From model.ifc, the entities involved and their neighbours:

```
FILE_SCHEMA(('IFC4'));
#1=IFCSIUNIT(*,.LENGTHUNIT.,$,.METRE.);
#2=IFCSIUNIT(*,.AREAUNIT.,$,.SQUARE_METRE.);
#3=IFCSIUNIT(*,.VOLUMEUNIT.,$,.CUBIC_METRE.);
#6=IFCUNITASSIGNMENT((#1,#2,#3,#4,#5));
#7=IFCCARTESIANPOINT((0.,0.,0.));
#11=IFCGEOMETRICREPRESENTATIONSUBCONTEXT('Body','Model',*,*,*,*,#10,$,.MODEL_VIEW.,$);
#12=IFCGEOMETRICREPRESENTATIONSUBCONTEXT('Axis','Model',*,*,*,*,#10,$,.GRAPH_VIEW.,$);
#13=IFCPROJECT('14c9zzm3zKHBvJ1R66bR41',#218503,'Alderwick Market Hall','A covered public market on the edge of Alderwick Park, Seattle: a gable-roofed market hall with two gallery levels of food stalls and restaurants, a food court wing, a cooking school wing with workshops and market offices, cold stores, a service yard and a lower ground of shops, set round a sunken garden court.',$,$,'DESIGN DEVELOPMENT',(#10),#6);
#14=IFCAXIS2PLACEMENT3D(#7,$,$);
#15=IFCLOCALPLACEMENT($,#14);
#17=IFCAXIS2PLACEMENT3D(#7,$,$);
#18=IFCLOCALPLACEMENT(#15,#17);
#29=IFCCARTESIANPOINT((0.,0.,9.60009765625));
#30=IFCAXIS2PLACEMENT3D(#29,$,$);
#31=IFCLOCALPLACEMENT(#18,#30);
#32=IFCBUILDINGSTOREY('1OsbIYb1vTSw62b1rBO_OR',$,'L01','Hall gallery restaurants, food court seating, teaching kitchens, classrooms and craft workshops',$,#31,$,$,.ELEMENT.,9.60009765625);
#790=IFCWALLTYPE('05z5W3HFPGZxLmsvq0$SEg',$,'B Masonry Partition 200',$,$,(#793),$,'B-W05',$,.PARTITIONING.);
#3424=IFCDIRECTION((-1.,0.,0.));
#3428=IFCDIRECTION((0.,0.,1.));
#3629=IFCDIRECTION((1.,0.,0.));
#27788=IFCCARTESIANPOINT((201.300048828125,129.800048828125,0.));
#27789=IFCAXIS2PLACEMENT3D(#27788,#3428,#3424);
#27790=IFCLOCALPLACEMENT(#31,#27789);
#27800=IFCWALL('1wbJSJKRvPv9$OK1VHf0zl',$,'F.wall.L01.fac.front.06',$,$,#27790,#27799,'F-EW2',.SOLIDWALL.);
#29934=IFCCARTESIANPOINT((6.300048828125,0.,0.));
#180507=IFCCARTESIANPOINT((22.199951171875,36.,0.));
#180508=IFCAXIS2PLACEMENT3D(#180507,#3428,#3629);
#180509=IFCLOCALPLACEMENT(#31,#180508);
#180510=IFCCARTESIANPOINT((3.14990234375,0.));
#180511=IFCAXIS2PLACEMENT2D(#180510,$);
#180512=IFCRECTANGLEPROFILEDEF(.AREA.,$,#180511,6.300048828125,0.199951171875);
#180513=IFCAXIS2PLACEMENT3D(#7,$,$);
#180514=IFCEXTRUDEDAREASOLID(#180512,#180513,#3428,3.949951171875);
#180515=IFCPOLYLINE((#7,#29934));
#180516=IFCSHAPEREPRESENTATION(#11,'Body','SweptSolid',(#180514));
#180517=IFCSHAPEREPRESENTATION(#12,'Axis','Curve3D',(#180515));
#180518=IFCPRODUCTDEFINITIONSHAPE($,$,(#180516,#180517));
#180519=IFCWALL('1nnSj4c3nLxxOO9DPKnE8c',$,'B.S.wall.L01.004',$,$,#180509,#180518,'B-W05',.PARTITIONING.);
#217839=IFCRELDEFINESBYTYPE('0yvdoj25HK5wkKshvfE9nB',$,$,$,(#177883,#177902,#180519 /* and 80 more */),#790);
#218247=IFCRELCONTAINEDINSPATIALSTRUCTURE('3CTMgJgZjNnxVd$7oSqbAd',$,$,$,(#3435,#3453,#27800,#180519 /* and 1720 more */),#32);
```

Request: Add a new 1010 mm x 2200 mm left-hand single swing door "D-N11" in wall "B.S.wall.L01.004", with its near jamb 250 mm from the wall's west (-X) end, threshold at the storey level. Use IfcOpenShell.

```python
import numpy as np
import ifcopenshell
import ifcopenshell.api.feature
import ifcopenshell.api.geometry
import ifcopenshell.api.root
import ifcopenshell.api.spatial
import ifcopenshell.geom
import ifcopenshell.util.element
import ifcopenshell.util.placement
import ifcopenshell.util.representation
import ifcopenshell.util.shape
import ifcopenshell.util.unit

model = ifcopenshell.open("model.ifc")
unit_scale = ifcopenshell.util.unit.calculate_unit_scale(model)
settings = ifcopenshell.geom.settings()


def volume(element):
    """Net volume in cubic metres, openings subtracted."""
    shape = ifcopenshell.geom.create_shape(settings, element)
    return ifcopenshell.util.shape.get_volume(shape.geometry)


wall = model.by_guid("1nnSj4c3nLxxOO9DPKnE8c")
storey = ifcopenshell.util.element.get_container(wall, ifc_class="IfcBuildingStorey")
context = ifcopenshell.util.representation.get_context(model, "Model", "Body", "MODEL_VIEW")
before = volume(wall)

width, height, from_end, sill = 1.01, 2.2, 0.25, 0.0  # metres

# The wall runs along its own X axis, and the end named is its -X end.
wall_shape = ifcopenshell.geom.create_shape(settings, wall)
x, y, z = ifcopenshell.util.shape.get_vertices(wall_shape.geometry).T
start = x.min() + from_end
face, thickness = float(y.min()), float(y.max() - y.min())
wall_matrix = ifcopenshell.util.placement.get_local_placement(wall.ObjectPlacement)
level = ifcopenshell.util.placement.get_local_placement(storey.ObjectPlacement)[2, 3]


def in_wall(x, y):
    """Placement at x, y metres in the wall's axes, at sill height."""
    matrix = wall_matrix.copy()
    matrix[:, 3] = wall_matrix @ np.array([x / unit_scale, y / unit_scale, 0.0, 1.0])
    matrix[2, 3] = level + sill / unit_scale
    return matrix


# Opening: a box that overshoots both wall faces by 50 mm.
opening = ifcopenshell.api.root.create_entity(model, ifc_class="IfcOpeningElement", predefined_type="OPENING")
box = ifcopenshell.api.geometry.add_wall_representation(
    model, context=context, length=width, height=height, thickness=thickness + 0.1
)
ifcopenshell.api.geometry.assign_representation(model, product=opening, representation=box)
ifcopenshell.api.geometry.edit_object_placement(model, product=opening, matrix=in_wall(start, face - 0.05), is_si=False)
ifcopenshell.api.feature.add_feature(model, feature=opening, element=wall)

door = ifcopenshell.api.root.create_entity(model, ifc_class="IfcDoor", name="D-N11", predefined_type="DOOR")
door.OverallWidth, door.OverallHeight = width / unit_scale, height / unit_scale
door.OperationType = "SINGLE_SWING_LEFT"
body = ifcopenshell.api.geometry.add_door_representation(
    model,
    context=context,
    overall_width=door.OverallWidth,
    overall_height=door.OverallHeight,
    operation_type="SINGLE_SWING_LEFT",
    lining_properties={"LiningDepth": thickness / unit_scale, "ThresholdDepth": thickness / unit_scale},
)
ifcopenshell.api.geometry.assign_representation(model, product=door, representation=body)
ifcopenshell.api.spatial.assign_container(model, products=[door], relating_structure=storey)
ifcopenshell.api.feature.add_filling(model, opening=opening, element=door)

# The lining spans the wall, so the door starts at the wall face.
ifcopenshell.api.geometry.edit_object_placement(model, product=door, matrix=in_wall(start, face), is_si=False)

after = volume(wall)

print(f"wall volume {before:.3f} -> {after:.3f} m3")

model.write("model_edited.ifc")
```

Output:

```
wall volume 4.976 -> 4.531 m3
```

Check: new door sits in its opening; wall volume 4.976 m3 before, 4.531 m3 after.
